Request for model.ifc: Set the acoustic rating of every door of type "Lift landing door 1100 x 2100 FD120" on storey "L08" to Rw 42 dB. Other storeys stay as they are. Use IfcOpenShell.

First a look at what the model holds.

```python
import ifcopenshell
import ifcopenshell.util.element

model = ifcopenshell.open("model.ifc")
print(model.schema)
storey = next(s for s in model.by_type("IfcBuildingStorey") if s.Name == "L08")
doors = [e for e in ifcopenshell.util.element.get_decomposition(storey) if e.is_a("IfcDoor")]
seen = {}
for e in doors:
    element_type = ifcopenshell.util.element.get_type(e)
    key = (element_type.Name if element_type != e and element_type else None, ifcopenshell.util.element.get_pset(e, "Pset_DoorCommon", "AcousticRating"))
    seen[key] = seen.get(key, 0) + 1
for (name, value), count in sorted(seen.items(), key=str):
    print(count, "x", name, "|", value)
```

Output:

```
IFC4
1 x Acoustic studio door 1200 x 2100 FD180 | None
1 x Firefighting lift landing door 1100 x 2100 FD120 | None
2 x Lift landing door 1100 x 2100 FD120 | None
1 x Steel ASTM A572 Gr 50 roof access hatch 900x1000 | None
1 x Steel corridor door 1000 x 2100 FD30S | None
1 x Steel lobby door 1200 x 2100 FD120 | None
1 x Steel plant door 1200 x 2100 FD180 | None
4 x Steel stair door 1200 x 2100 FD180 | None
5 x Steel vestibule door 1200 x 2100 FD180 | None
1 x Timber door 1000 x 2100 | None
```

```python
import ifcopenshell
import ifcopenshell.api.pset
import ifcopenshell.util.element

model = ifcopenshell.open("model.ifc")

storey = next(s for s in model.by_type("IfcBuildingStorey") if s.Name == "L08")
doors = [e for e in ifcopenshell.util.element.get_decomposition(storey) if e.is_a("IfcDoor")]

count = 0
for e in doors:
    element_type = ifcopenshell.util.element.get_type(e)
    if element_type in (None, e) or element_type.Name != "Lift landing door 1100 x 2100 FD120":
        continue
    # add_pset returns the element's existing set when there is one.
    pset = ifcopenshell.api.pset.add_pset(model, product=e, name="Pset_DoorCommon")
    ifcopenshell.api.pset.edit_pset(model, pset=pset, properties={"AcousticRating": "Rw 42 dB"})
    count += 1

print(count, "doors updated")

model.write("model_edited.ifc")
```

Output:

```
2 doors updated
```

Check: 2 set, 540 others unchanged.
